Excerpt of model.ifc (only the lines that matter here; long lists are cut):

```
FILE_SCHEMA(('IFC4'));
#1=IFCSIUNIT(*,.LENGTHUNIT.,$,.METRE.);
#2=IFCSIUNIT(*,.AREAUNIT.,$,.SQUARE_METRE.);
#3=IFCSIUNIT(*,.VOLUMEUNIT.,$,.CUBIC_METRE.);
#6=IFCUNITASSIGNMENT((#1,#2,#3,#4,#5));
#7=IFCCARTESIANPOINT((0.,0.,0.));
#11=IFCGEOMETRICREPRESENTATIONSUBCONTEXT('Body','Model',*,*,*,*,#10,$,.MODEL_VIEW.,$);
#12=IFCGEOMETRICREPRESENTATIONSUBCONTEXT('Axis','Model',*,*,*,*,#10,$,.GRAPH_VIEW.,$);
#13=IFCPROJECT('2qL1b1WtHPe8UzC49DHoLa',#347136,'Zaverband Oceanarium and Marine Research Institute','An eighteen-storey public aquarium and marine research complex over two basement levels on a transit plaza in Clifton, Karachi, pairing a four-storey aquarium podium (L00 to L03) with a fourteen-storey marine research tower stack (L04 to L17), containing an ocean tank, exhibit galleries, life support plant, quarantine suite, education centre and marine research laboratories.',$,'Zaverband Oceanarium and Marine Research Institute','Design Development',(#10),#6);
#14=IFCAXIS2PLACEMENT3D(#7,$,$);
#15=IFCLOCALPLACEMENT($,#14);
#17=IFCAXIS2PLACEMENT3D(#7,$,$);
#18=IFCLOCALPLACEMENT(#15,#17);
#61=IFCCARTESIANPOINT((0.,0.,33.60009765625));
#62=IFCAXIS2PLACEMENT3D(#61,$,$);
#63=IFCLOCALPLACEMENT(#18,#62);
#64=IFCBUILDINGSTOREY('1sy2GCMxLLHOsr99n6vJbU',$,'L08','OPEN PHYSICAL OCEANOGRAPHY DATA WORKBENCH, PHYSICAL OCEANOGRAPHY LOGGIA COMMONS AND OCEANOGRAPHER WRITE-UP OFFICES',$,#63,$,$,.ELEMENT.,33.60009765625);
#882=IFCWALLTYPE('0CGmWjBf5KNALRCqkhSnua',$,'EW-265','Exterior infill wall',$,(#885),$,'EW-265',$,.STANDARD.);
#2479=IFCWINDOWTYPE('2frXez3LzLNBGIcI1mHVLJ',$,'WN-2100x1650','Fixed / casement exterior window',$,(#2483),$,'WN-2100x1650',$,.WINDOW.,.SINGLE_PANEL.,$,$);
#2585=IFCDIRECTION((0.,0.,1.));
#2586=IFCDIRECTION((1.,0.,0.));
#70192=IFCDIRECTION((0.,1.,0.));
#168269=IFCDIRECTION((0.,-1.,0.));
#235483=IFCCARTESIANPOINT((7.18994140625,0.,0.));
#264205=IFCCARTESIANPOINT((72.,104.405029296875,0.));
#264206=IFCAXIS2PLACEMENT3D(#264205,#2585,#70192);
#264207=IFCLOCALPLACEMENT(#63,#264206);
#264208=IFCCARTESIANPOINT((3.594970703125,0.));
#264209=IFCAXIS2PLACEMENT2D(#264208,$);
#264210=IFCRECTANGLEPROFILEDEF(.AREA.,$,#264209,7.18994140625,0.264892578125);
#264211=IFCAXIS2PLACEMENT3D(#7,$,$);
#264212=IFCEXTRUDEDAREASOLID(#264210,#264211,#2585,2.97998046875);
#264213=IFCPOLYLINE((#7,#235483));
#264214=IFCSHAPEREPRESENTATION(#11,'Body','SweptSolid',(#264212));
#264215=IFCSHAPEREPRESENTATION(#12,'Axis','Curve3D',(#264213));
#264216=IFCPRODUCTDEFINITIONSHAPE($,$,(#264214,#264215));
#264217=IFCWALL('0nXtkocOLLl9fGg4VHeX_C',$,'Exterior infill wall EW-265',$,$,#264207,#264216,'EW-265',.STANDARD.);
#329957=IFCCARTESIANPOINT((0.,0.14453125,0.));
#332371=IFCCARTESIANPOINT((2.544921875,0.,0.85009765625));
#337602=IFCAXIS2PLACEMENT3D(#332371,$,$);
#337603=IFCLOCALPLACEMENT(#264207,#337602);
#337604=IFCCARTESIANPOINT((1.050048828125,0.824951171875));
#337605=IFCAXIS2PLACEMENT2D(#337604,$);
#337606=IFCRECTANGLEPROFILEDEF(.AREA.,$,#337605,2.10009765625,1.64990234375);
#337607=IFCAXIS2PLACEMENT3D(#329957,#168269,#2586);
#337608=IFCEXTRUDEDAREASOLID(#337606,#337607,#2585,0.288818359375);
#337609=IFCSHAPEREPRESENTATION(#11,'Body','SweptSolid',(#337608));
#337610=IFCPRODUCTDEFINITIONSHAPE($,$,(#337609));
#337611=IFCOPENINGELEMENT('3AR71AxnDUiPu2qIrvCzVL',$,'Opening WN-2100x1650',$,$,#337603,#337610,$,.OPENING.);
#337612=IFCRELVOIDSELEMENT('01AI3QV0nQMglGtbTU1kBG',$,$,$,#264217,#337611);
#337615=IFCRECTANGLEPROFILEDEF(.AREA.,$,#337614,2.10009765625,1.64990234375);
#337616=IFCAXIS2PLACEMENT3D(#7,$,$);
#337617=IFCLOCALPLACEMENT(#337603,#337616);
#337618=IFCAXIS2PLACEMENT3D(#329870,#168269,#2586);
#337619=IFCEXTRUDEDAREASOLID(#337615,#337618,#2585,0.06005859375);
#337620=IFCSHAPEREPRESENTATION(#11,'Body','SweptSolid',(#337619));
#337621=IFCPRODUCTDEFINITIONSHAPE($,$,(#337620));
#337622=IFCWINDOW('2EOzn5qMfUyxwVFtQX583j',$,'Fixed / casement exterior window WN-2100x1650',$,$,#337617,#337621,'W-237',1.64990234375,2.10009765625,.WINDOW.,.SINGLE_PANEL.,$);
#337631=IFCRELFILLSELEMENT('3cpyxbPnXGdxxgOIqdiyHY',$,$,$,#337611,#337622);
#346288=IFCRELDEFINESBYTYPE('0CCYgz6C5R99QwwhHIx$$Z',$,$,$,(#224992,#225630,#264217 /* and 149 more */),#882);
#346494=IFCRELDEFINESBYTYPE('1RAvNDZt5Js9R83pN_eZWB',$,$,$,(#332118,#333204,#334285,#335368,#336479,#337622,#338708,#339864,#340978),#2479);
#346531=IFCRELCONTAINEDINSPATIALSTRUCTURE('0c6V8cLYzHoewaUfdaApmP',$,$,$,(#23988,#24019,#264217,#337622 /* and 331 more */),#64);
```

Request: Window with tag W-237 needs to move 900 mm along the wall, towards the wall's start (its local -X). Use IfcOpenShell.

```python
import ifcopenshell
import ifcopenshell.api.geometry
import ifcopenshell.util.placement
import ifcopenshell.util.unit

model = ifcopenshell.open("model.ifc")
unit_scale = ifcopenshell.util.unit.calculate_unit_scale(model)

window = model.by_id(337622)
opening = window.FillsVoids[0].RelatingOpeningElement
wall = opening.VoidsElements[0].RelatingBuildingElement

wall_matrix = ifcopenshell.util.placement.get_local_placement(wall.ObjectPlacement)
shift = wall_matrix[:3, 0] * -0.9 / unit_scale
before = ifcopenshell.util.placement.get_local_placement(window.ObjectPlacement)[:3, 3].copy()

# The window is placed relative to its opening, so it follows when the opening moves.
matrix = ifcopenshell.util.placement.get_local_placement(opening.ObjectPlacement)
matrix[:3, 3] += shift
ifcopenshell.api.geometry.edit_object_placement(
    model, product=opening, matrix=matrix, is_si=False, should_transform_children=True
)

after = ifcopenshell.util.placement.get_local_placement(window.ObjectPlacement)[:3, 3]
print("window moved by", (after - before).round(3) + 0.0)

model.write("model_rev.ifc")
```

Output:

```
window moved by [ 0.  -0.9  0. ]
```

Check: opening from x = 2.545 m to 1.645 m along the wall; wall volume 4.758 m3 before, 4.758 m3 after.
